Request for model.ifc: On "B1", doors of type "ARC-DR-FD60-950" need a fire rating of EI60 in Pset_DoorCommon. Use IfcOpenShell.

First a look at what the model holds.

```python
import ifcopenshell
import ifcopenshell.util.element

model = ifcopenshell.open("model.ifc")
print(model.schema)
storey = next(s for s in model.by_type("IfcBuildingStorey") if s.Name == "B1")
doors = [e for e in ifcopenshell.util.element.get_decomposition(storey) if e.is_a("IfcDoor")]
seen = {}
for e in doors:
    element_type = ifcopenshell.util.element.get_type(e)
    key = (element_type.Name if element_type != e and element_type else None, ifcopenshell.util.element.get_pset(e, "Pset_DoorCommon", "FireRating"))
    seen[key] = seen.get(key, 0) + 1
for (name, value), count in sorted(seen.items(), key=str):
    print(count, "x", name, "|", value)
```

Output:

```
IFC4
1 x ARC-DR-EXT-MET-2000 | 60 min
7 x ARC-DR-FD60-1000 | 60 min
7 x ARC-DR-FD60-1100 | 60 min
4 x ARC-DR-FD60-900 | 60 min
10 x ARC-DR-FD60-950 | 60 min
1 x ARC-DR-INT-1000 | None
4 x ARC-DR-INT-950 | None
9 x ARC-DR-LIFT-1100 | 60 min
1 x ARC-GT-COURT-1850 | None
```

```python
import ifcopenshell
import ifcopenshell.api.pset
import ifcopenshell.util.element

model = ifcopenshell.open("model.ifc")

storey = next(s for s in model.by_type("IfcBuildingStorey") if s.Name == "B1")
doors = [e for e in ifcopenshell.util.element.get_decomposition(storey) if e.is_a("IfcDoor")]

count = 0
for e in doors:
    element_type = ifcopenshell.util.element.get_type(e)
    if element_type in (None, e) or element_type.Name != "ARC-DR-FD60-950":
        continue
    # add_pset returns the element's existing set when there is one.
    pset = ifcopenshell.api.pset.add_pset(model, product=e, name="Pset_DoorCommon")
    ifcopenshell.api.pset.edit_pset(model, pset=pset, properties={"FireRating": "EI60"})
    count += 1

print(count, "doors updated")

model.write("model_edited.ifc")
```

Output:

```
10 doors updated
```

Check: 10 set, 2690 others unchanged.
